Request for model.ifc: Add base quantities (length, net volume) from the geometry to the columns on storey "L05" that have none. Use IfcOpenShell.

First a look at what the model holds.

```python
import ifcopenshell
import ifcopenshell.util.element
import ifcopenshell.util.unit

model = ifcopenshell.open("model.ifc")
print(model.schema)
for unit_type in ("LENGTHUNIT", "AREAUNIT", "VOLUMEUNIT"):
    print(unit_type, ifcopenshell.util.unit.calculate_unit_scale(model, unit_type))
storey = next(s for s in model.by_type("IfcBuildingStorey") if s.Name == "L05")
columns = [e for e in ifcopenshell.util.element.get_decomposition(storey) if e.is_a("IfcColumn")]
for e in sorted(columns, key=lambda e: e.id()):
    print(e.id(), e.is_a(), e.Name, list(ifcopenshell.util.element.get_psets(e, qtos_only=True)), sep=" | ")
```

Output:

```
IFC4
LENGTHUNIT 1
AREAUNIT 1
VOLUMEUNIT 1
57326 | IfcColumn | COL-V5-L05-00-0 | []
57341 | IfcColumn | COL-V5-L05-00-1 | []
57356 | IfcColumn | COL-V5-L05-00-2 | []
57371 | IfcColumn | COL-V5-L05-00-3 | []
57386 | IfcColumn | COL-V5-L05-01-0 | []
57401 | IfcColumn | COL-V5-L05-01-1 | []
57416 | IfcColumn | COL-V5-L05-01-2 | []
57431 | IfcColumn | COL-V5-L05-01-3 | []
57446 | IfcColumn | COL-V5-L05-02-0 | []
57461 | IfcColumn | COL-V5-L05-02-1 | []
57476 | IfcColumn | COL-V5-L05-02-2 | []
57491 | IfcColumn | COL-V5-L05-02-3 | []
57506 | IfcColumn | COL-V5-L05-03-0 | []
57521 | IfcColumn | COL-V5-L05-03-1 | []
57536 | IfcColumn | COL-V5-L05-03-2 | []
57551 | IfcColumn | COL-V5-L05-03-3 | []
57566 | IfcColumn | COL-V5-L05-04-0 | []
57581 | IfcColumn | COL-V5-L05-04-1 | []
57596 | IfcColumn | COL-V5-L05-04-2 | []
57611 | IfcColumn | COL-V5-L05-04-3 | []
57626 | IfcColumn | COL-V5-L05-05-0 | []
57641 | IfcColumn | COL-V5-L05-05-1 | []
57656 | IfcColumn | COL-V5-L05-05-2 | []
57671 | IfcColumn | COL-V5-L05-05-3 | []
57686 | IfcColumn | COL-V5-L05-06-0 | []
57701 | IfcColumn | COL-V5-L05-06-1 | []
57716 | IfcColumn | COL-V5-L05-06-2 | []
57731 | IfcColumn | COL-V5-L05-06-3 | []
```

```python
import ifcopenshell
import ifcopenshell.api.pset
import ifcopenshell.geom
import ifcopenshell.util.element
import ifcopenshell.util.shape
import ifcopenshell.util.unit

model = ifcopenshell.open("model.ifc")
unit_scale = ifcopenshell.util.unit.calculate_unit_scale(model)
volume_scale = ifcopenshell.util.unit.calculate_unit_scale(model, "VOLUMEUNIT")
settings = ifcopenshell.geom.settings()

storey = next(s for s in model.by_type("IfcBuildingStorey") if s.Name == "L05")
columns = [e for e in ifcopenshell.util.element.get_decomposition(storey) if e.is_a("IfcColumn")]

for e in sorted(columns, key=lambda e: e.id()):
    if ifcopenshell.util.element.get_psets(e, qtos_only=True, should_inherit=False):
        continue
    # Geometry comes back in metres, in the element's own axes.
    shape = ifcopenshell.geom.create_shape(settings, e)
    values = {
        "Length": ifcopenshell.util.shape.get_z(shape.geometry) / unit_scale,
        "NetVolume": ifcopenshell.util.shape.get_volume(shape.geometry) / volume_scale,
    }
    qto = ifcopenshell.api.pset.add_qto(model, product=e, name="Qto_ColumnBaseQuantities")
    ifcopenshell.api.pset.edit_qto(model, qto=qto, properties=values)
    print(e.id(), {k: round(v, 3) for k, v in values.items()})

model.write("model_edited.ifc")
```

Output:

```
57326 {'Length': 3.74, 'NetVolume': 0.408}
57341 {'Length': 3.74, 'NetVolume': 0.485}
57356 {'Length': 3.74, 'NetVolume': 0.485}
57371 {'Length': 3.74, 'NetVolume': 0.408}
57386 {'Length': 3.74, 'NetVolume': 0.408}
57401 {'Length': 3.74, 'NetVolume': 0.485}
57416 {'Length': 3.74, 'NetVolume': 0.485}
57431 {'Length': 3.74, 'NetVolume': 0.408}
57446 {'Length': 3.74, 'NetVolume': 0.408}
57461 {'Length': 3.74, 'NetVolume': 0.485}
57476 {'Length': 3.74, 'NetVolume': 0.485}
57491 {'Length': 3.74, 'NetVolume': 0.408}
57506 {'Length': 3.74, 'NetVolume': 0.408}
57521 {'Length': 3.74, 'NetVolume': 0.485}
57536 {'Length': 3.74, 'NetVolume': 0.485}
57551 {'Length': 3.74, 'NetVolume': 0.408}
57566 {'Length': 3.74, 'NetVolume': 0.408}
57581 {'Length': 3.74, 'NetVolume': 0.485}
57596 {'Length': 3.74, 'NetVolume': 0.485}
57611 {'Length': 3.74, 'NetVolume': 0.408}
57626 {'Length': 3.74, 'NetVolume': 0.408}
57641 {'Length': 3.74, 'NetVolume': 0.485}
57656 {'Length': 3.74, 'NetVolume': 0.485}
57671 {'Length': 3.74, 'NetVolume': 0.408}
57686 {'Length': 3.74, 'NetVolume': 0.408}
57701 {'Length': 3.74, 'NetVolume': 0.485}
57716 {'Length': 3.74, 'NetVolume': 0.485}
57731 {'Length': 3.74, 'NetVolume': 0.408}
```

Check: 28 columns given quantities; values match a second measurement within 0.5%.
